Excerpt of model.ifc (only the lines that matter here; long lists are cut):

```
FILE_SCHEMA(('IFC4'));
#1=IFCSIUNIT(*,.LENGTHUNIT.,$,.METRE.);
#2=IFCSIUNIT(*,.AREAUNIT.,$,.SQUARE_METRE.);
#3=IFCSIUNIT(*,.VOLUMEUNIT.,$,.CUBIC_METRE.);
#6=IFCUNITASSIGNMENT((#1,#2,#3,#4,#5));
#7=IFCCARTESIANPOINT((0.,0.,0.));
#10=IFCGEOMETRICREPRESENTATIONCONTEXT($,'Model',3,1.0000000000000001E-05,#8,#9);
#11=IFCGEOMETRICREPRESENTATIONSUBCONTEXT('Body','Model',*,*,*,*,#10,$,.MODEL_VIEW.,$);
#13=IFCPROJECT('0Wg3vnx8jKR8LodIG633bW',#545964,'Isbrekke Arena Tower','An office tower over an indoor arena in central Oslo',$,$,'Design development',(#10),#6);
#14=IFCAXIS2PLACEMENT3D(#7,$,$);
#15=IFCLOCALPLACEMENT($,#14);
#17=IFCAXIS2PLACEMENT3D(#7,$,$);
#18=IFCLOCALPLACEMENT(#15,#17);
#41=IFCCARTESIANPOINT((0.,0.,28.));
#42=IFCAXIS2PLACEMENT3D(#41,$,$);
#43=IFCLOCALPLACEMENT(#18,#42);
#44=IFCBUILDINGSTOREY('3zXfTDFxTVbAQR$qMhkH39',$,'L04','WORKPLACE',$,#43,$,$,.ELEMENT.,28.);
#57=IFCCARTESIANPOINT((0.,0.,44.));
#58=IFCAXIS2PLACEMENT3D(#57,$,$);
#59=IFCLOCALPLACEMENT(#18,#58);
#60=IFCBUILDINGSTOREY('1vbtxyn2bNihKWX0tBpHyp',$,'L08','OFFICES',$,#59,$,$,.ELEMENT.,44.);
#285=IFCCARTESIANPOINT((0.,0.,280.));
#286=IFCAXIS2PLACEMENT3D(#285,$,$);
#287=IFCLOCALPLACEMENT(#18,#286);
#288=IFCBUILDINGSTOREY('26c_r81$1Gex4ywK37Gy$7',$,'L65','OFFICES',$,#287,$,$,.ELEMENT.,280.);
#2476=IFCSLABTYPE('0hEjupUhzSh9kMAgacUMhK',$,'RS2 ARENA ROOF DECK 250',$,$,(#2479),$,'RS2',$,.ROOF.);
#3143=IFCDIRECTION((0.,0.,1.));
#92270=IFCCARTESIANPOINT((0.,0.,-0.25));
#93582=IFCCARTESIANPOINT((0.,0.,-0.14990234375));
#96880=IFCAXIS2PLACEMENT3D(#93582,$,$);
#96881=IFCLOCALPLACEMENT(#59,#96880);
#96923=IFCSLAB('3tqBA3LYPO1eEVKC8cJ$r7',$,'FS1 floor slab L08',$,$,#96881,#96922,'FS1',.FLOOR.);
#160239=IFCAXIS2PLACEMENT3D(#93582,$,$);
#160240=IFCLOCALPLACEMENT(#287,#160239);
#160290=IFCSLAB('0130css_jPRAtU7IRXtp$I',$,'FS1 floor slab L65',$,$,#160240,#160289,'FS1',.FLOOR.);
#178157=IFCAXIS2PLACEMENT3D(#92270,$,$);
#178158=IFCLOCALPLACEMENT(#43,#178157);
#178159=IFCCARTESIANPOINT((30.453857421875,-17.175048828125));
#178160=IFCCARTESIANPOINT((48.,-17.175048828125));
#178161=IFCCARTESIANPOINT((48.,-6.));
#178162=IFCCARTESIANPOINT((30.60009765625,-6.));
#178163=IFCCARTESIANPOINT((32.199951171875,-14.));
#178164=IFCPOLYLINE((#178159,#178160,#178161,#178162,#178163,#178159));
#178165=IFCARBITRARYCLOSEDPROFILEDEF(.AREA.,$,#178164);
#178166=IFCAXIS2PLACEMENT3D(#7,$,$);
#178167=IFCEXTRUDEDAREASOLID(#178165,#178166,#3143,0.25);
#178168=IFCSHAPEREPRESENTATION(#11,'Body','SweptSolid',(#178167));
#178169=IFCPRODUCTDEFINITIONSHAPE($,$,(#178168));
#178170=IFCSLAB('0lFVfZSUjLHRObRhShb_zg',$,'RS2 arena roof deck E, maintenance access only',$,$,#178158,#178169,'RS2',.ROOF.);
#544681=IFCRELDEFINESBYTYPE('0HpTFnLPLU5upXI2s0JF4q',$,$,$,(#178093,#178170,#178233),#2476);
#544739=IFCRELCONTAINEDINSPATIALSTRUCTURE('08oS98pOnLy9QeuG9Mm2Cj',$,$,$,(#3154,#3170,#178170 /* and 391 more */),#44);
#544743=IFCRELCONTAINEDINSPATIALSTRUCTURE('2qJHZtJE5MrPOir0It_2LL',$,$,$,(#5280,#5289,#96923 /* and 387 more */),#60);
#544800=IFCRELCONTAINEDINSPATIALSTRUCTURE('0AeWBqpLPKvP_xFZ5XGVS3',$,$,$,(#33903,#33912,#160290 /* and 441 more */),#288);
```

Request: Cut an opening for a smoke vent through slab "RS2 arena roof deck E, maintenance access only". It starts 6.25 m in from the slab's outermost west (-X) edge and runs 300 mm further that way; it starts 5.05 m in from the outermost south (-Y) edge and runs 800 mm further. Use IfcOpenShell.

```python
import numpy as np
import ifcopenshell
import ifcopenshell.api.feature
import ifcopenshell.api.geometry
import ifcopenshell.api.root
import ifcopenshell.geom
import ifcopenshell.util.placement
import ifcopenshell.util.representation
import ifcopenshell.util.shape
import ifcopenshell.util.unit

model = ifcopenshell.open("model.ifc")
unit_scale = ifcopenshell.util.unit.calculate_unit_scale(model)
settings = ifcopenshell.geom.settings()


def volume(element):
    """Net volume in cubic metres, openings subtracted."""
    shape = ifcopenshell.geom.create_shape(settings, element)
    return ifcopenshell.util.shape.get_volume(shape.geometry)


slab = model.by_guid("0lFVfZSUjLHRObRhShb_zg")
before = volume(slab)

# Extent in the slab's own axes, in metres. The edges named are its -X and -Y sides.
slab_shape = ifcopenshell.geom.create_shape(settings, slab)
vertices = ifcopenshell.util.shape.get_vertices(slab_shape.geometry)
x_min, y_min, bottom = vertices.min(axis=0)
top = vertices[:, 2].max()

opening = ifcopenshell.api.root.create_entity(model, ifc_class="IfcOpeningElement", name="Smoke vent opening", predefined_type="OPENING")
context = ifcopenshell.util.representation.get_context(model, "Model", "Body", "MODEL_VIEW")
width, depth = 0.3, 0.8
outline = [(0.0, 0.0), (width, 0.0), (width, depth), (0.0, depth), (0.0, 0.0)]
# Overshoot both faces by 50 mm so the cut is clean.
shape = ifcopenshell.api.geometry.add_slab_representation(
    model, context=context, depth=top - bottom + 0.1, polyline=outline
)
ifcopenshell.api.geometry.assign_representation(model, product=opening, representation=shape)

matrix = ifcopenshell.util.placement.get_local_placement(slab.ObjectPlacement)
matrix[:, 3] = matrix @ np.append(np.array([x_min + 6.25, y_min + 5.05, bottom - 0.05]) / unit_scale, 1.0)
ifcopenshell.api.geometry.edit_object_placement(model, product=opening, matrix=matrix, is_si=False)
ifcopenshell.api.feature.add_feature(model, feature=opening, element=slab)

after = volume(slab)

print(f"slab volume {before:.3f} -> {after:.3f} m3")

model.write("model_updated.ifc")
```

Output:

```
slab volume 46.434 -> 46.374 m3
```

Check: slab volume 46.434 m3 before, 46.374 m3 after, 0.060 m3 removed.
